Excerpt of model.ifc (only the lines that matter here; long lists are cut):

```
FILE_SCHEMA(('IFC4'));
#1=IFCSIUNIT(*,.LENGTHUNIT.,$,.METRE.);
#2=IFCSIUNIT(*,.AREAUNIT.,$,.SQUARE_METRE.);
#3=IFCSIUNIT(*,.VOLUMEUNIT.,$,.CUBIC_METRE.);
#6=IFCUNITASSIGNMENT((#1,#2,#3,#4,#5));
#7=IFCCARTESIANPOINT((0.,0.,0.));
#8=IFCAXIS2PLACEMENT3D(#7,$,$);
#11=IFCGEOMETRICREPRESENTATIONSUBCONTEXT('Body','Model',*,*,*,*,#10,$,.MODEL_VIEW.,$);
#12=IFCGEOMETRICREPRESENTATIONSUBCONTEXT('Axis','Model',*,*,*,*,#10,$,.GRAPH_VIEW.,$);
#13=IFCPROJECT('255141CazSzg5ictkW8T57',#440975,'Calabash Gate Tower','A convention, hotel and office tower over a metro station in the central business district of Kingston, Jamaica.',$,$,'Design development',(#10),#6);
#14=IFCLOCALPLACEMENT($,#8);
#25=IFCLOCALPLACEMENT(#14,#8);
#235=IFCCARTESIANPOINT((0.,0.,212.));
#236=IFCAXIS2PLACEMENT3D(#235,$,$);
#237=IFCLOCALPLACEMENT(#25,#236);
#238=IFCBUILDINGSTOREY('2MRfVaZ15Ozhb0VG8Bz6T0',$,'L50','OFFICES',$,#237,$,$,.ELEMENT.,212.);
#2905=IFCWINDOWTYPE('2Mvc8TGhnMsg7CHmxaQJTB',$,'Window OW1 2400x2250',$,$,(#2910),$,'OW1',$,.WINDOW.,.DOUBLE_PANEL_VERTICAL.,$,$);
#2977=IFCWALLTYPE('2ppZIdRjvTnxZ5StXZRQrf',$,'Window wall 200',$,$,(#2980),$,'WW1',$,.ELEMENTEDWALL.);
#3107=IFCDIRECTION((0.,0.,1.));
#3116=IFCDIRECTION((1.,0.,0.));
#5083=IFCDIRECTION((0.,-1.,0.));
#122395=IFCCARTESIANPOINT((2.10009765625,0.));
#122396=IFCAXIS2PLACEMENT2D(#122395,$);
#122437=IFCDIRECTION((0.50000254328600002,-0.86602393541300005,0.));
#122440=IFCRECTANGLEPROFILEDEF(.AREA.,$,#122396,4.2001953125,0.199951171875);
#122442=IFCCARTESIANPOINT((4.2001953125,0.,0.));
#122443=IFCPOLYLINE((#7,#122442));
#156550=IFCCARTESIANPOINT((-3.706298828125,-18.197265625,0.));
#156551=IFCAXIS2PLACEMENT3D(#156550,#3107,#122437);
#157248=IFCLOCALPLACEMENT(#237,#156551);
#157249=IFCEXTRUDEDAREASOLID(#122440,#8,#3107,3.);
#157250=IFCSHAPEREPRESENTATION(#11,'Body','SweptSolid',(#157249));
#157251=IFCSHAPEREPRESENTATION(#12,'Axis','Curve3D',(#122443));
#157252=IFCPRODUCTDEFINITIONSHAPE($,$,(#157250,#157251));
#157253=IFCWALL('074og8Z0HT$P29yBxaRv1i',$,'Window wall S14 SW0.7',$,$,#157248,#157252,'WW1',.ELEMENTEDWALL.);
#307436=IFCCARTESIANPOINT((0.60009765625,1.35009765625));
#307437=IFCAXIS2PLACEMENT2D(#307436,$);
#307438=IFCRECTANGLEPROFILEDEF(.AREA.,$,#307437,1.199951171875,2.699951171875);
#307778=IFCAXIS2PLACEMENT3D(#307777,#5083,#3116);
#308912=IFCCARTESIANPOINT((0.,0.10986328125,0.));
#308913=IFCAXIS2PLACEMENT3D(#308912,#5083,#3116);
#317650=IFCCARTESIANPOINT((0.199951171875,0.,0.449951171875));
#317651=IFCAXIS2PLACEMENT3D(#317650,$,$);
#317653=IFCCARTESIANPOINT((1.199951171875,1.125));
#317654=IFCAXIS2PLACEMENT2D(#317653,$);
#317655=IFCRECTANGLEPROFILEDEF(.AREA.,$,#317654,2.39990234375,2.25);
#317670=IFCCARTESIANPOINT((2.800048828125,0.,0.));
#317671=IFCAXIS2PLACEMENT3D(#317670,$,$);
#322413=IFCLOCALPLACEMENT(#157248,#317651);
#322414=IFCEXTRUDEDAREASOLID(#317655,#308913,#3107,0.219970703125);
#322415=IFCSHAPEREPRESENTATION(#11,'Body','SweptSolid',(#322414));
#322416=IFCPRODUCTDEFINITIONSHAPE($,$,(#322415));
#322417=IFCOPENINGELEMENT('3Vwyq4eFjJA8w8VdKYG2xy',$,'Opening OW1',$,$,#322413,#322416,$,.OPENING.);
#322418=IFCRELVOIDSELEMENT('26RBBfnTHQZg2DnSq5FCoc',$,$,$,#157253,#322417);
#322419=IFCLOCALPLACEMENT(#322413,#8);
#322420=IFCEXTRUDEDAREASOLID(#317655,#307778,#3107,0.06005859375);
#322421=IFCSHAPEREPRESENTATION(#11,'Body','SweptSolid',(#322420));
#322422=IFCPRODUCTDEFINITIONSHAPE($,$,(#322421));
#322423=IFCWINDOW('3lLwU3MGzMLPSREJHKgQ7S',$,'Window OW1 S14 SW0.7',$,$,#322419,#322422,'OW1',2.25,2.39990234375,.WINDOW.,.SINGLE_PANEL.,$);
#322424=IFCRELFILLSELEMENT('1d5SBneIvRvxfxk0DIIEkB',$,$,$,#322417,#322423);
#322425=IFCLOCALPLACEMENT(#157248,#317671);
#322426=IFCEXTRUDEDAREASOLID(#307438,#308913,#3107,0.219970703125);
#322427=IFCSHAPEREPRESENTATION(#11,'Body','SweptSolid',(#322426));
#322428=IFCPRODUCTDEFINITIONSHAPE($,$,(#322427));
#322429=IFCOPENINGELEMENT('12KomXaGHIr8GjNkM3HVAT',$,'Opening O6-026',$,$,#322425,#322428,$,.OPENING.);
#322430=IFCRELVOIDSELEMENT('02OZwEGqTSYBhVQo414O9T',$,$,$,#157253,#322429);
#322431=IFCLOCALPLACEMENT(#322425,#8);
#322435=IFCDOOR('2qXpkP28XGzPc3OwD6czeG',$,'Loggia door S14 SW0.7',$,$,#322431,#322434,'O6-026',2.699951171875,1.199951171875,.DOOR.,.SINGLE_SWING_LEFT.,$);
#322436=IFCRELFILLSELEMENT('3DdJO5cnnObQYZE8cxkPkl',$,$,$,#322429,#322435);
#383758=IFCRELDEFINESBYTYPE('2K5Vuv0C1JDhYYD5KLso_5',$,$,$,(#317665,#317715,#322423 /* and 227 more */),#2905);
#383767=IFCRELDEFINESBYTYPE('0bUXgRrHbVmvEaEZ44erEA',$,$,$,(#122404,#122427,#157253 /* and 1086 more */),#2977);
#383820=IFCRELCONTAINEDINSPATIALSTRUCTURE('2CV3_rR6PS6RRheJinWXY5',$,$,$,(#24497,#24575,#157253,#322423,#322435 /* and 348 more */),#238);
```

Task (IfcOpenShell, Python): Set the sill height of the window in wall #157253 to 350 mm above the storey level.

```python
import numpy as np
import ifcopenshell
import ifcopenshell.api.geometry
import ifcopenshell.geom
import ifcopenshell.util.element
import ifcopenshell.util.placement
import ifcopenshell.util.shape
import ifcopenshell.util.unit

model = ifcopenshell.open("model.ifc")
unit_scale = ifcopenshell.util.unit.calculate_unit_scale(model)

window = model.by_guid("3lLwU3MGzMLPSREJHKgQ7S")
opening = window.FillsVoids[0].RelatingOpeningElement
storey = ifcopenshell.util.element.get_container(window, ifc_class="IfcBuildingStorey")
level = ifcopenshell.util.placement.get_local_placement(storey.ObjectPlacement)[2, 3]

# The opening's origin need not be at the sill, so measure its lowest point.
shape = ifcopenshell.geom.create_shape(ifcopenshell.geom.settings(), opening)
bottom = ifcopenshell.util.shape.get_shape_bottom_elevation(shape, shape.geometry) / unit_scale
dz = level + 0.35 / unit_scale - bottom

shift = np.array([0.0, 0.0, dz])
# The window is placed relative to its opening, so it follows when the opening moves.
matrix = ifcopenshell.util.placement.get_local_placement(opening.ObjectPlacement)
matrix[:3, 3] += shift
ifcopenshell.api.geometry.edit_object_placement(
    model, product=opening, matrix=matrix, is_si=False, should_transform_children=True
)

print(f"moved by {dz * unit_scale:+.3f} m")

model.write("model-out.ifc")
```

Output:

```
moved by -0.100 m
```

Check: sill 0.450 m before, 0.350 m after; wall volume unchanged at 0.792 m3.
